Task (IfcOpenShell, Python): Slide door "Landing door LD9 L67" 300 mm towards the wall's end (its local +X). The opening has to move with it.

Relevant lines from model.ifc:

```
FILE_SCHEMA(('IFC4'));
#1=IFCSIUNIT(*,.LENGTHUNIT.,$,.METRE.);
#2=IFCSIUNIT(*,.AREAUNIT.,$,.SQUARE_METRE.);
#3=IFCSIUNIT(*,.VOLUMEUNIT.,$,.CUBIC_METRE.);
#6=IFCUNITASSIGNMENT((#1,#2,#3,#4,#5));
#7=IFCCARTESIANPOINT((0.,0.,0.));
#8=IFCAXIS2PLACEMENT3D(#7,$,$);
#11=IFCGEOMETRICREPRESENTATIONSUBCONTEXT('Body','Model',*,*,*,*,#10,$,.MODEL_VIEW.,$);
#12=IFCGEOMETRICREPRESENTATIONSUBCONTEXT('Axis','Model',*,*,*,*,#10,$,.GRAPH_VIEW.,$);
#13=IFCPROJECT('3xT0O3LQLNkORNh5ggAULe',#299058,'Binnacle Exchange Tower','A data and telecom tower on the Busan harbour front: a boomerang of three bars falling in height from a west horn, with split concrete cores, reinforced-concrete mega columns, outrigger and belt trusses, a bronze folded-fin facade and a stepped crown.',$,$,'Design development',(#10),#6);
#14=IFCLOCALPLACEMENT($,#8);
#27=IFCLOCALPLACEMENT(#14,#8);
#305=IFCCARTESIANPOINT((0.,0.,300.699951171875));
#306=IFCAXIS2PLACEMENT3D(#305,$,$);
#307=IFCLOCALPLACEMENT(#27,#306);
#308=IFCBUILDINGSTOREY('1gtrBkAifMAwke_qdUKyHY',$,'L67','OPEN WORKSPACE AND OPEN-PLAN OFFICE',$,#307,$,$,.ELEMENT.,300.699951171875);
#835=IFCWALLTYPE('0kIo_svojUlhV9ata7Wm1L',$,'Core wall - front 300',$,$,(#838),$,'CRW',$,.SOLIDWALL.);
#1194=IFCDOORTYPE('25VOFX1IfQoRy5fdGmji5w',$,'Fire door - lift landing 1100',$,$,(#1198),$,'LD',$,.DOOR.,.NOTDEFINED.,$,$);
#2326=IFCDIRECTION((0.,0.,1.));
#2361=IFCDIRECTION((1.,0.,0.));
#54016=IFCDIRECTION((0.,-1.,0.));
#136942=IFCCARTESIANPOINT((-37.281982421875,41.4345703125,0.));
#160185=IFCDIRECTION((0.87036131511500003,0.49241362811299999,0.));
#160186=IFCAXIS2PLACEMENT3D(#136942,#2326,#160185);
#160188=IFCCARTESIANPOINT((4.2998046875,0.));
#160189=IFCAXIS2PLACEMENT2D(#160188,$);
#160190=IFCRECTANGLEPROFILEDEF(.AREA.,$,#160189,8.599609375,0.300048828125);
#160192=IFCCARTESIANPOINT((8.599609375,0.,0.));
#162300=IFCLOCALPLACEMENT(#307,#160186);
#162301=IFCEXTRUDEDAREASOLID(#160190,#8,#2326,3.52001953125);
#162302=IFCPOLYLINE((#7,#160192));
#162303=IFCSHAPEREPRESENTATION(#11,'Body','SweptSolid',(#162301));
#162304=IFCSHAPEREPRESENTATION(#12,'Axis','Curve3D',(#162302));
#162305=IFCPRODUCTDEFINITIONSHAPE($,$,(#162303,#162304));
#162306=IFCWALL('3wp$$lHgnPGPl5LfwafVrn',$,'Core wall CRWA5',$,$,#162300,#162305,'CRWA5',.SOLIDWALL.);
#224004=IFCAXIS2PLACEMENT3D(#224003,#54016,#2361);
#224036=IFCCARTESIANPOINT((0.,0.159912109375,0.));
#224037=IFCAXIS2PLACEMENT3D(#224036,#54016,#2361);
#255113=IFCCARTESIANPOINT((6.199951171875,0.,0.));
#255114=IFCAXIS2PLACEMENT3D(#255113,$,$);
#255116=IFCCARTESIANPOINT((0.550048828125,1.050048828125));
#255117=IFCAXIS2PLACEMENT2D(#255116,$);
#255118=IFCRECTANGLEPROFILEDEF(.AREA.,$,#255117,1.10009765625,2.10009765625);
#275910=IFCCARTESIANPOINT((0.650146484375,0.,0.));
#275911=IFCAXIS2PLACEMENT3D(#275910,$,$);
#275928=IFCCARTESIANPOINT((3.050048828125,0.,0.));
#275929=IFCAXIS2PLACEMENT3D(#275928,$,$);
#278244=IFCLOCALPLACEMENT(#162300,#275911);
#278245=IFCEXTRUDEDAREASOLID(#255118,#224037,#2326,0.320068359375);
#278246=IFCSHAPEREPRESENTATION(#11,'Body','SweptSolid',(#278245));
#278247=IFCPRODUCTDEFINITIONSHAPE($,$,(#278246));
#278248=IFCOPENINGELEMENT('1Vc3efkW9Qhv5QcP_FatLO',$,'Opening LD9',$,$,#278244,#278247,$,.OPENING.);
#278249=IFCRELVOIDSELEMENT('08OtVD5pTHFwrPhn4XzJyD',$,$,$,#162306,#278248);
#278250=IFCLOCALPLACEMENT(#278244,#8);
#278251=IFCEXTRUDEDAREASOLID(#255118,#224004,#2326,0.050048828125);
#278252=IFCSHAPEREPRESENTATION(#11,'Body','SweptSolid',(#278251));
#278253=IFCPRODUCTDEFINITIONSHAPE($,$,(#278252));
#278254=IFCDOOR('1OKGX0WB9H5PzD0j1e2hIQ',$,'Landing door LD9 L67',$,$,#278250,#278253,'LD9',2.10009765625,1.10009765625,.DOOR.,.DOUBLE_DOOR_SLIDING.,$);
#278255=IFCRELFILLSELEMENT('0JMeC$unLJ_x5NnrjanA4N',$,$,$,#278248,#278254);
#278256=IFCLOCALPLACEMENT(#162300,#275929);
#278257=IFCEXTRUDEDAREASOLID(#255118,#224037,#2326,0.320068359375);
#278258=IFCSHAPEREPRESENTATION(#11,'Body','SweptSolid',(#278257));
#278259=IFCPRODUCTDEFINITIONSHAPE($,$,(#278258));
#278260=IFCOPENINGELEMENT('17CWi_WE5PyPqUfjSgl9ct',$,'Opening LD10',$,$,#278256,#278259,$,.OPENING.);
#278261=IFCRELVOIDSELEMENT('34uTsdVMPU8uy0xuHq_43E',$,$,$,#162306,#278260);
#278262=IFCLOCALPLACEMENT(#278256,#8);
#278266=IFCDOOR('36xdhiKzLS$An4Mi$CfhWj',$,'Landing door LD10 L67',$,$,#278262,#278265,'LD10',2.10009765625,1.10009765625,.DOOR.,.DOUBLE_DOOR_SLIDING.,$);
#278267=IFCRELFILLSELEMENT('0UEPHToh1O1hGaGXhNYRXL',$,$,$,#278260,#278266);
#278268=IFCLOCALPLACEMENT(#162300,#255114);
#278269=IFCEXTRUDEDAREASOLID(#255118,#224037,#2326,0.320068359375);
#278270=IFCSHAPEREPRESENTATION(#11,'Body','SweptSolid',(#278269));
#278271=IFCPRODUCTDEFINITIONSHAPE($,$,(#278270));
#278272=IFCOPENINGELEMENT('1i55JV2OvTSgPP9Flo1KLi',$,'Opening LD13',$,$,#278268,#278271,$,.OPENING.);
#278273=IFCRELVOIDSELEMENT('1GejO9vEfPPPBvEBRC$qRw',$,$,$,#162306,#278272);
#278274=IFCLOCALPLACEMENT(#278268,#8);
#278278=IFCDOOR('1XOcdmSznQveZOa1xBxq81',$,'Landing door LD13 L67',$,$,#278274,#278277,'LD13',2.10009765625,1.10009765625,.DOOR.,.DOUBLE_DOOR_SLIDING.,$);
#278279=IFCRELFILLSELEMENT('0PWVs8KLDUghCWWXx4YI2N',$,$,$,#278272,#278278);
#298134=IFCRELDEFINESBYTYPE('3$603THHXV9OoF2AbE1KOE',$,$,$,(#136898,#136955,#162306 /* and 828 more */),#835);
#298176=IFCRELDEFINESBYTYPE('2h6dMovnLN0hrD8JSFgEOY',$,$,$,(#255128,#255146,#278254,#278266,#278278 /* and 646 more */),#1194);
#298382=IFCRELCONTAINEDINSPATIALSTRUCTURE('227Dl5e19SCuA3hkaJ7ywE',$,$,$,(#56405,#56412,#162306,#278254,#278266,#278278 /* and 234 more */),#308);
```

```python
import ifcopenshell
import ifcopenshell.api.geometry
import ifcopenshell.util.placement
import ifcopenshell.util.unit

model = ifcopenshell.open("model.ifc")
unit_scale = ifcopenshell.util.unit.calculate_unit_scale(model)

door = model.by_id(278254)
opening = door.FillsVoids[0].RelatingOpeningElement
wall = opening.VoidsElements[0].RelatingBuildingElement

wall_matrix = ifcopenshell.util.placement.get_local_placement(wall.ObjectPlacement)
shift = wall_matrix[:3, 0] * 0.3 / unit_scale
before = ifcopenshell.util.placement.get_local_placement(door.ObjectPlacement)[:3, 3].copy()

# The door is placed relative to its opening, so it follows when the opening moves.
matrix = ifcopenshell.util.placement.get_local_placement(opening.ObjectPlacement)
matrix[:3, 3] += shift
ifcopenshell.api.geometry.edit_object_placement(
    model, product=opening, matrix=matrix, is_si=False, should_transform_children=True
)

after = ifcopenshell.util.placement.get_local_placement(door.ObjectPlacement)[:3, 3]
print("door moved by", (after - before).round(3) + 0.0)

model.write("model_v2.ifc")
```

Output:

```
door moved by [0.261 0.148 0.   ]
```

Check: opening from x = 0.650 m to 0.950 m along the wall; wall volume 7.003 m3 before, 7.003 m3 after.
